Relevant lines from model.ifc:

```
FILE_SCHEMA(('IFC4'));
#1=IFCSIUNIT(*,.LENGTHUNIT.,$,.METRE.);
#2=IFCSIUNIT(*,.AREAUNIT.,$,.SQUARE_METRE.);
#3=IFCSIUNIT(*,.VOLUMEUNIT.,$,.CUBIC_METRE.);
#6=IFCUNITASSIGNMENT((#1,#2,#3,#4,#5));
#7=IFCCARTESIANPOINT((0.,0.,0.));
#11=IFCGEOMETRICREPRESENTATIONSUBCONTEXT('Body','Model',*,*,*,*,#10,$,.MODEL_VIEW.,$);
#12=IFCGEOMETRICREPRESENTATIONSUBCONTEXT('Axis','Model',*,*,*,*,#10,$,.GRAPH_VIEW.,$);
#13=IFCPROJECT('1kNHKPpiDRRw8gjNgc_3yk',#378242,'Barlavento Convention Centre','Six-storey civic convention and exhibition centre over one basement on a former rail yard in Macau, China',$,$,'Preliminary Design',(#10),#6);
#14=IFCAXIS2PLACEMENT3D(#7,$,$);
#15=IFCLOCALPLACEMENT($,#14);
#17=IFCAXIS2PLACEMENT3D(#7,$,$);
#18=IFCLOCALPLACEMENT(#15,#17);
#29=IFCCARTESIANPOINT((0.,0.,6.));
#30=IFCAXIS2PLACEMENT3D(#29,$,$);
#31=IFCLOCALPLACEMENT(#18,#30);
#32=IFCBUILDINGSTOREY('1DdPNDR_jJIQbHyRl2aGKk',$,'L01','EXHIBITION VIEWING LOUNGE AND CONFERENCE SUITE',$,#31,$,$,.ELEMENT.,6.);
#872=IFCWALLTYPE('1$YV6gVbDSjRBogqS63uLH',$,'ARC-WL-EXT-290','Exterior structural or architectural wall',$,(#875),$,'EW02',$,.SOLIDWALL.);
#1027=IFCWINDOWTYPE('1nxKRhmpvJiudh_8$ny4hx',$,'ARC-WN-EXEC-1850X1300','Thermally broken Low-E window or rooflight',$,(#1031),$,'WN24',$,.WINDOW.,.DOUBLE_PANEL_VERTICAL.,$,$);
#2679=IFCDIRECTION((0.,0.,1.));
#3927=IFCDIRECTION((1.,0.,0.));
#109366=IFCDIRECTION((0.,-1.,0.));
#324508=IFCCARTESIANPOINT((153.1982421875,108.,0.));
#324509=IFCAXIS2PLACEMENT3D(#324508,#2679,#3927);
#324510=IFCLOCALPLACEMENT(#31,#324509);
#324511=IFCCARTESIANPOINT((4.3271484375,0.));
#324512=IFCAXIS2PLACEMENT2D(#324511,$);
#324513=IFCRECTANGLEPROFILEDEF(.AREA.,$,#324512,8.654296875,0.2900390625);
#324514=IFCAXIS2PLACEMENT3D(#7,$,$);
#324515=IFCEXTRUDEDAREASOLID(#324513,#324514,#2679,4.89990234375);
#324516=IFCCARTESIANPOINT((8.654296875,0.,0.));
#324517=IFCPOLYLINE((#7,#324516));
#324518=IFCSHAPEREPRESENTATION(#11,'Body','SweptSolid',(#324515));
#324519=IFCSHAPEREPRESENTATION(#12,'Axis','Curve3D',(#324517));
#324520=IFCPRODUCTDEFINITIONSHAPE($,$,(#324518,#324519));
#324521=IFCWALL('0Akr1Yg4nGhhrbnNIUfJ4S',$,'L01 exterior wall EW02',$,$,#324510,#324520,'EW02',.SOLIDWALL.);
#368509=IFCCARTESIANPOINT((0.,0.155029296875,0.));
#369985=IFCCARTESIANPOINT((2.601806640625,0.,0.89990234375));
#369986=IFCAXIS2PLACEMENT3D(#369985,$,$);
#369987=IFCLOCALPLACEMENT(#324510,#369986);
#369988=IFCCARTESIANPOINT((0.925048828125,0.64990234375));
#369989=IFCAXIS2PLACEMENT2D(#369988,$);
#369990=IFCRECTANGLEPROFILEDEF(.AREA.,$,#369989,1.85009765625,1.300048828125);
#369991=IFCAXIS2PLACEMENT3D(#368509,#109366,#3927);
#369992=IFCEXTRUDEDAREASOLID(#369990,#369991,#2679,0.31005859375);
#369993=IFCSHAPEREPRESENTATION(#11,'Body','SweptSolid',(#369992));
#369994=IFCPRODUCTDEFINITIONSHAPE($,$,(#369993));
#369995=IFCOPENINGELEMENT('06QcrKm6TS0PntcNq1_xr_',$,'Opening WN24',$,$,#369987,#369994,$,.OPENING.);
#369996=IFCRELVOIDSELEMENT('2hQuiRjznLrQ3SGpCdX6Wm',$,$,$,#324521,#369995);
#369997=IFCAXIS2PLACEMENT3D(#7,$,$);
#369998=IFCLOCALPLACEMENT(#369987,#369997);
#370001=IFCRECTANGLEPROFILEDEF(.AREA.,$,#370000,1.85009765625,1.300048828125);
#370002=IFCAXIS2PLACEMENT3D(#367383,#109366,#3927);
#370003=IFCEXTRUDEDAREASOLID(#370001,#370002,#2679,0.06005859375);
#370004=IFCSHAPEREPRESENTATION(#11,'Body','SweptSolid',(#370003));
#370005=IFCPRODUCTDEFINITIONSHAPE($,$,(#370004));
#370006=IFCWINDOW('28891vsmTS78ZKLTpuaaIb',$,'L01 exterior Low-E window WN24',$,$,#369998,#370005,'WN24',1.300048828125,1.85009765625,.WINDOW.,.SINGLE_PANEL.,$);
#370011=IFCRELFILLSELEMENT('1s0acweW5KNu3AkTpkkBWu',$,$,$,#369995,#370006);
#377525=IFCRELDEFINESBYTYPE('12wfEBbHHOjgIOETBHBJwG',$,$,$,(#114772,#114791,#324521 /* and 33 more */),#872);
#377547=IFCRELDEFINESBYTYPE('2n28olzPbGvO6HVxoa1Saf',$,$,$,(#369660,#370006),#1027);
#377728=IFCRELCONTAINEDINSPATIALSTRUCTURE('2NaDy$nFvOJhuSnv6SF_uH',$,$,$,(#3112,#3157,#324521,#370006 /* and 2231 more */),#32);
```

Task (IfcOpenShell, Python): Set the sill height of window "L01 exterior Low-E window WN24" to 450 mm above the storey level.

```python
import numpy as np
import ifcopenshell
import ifcopenshell.api.geometry
import ifcopenshell.geom
import ifcopenshell.util.element
import ifcopenshell.util.placement
import ifcopenshell.util.shape
import ifcopenshell.util.unit

model = ifcopenshell.open("model.ifc")
unit_scale = ifcopenshell.util.unit.calculate_unit_scale(model)

window = model.by_id(370006)
opening = window.FillsVoids[0].RelatingOpeningElement
storey = ifcopenshell.util.element.get_container(window, ifc_class="IfcBuildingStorey")
level = ifcopenshell.util.placement.get_local_placement(storey.ObjectPlacement)[2, 3]

# The opening's origin need not be at the sill, so measure its lowest point.
shape = ifcopenshell.geom.create_shape(ifcopenshell.geom.settings(), opening)
bottom = ifcopenshell.util.shape.get_shape_bottom_elevation(shape, shape.geometry) / unit_scale
dz = level + 0.45 / unit_scale - bottom

shift = np.array([0.0, 0.0, dz])
# The window is placed relative to its opening, so it follows when the opening moves.
matrix = ifcopenshell.util.placement.get_local_placement(opening.ObjectPlacement)
matrix[:3, 3] += shift
ifcopenshell.api.geometry.edit_object_placement(
    model, product=opening, matrix=matrix, is_si=False, should_transform_children=True
)

print(f"moved by {dz * unit_scale:+.3f} m")

model.write("model_edited.ifc")
```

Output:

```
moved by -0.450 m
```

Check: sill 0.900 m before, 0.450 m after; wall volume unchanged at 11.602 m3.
